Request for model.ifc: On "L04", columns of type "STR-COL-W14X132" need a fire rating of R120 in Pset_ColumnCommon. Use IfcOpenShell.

First a look at what the model holds.

```python
import ifcopenshell
import ifcopenshell.util.element

model = ifcopenshell.open("model.ifc")
print(model.schema)
storey = next(s for s in model.by_type("IfcBuildingStorey") if s.Name == "L04")
columns = [e for e in ifcopenshell.util.element.get_decomposition(storey) if e.is_a("IfcColumn")]
seen = {}
for e in columns:
    element_type = ifcopenshell.util.element.get_type(e)
    key = (element_type.Name if element_type != e and element_type else None, ifcopenshell.util.element.get_pset(e, "Pset_ColumnCommon", "FireRating"))
    seen[key] = seen.get(key, 0) + 1
for (name, value), count in sorted(seen.items(), key=str):
    print(count, "x", name, "|", value)
```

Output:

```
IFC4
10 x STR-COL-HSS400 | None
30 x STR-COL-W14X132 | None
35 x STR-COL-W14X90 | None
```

```python
import ifcopenshell
import ifcopenshell.api.pset
import ifcopenshell.util.element

model = ifcopenshell.open("model.ifc")

storey = next(s for s in model.by_type("IfcBuildingStorey") if s.Name == "L04")
columns = [e for e in ifcopenshell.util.element.get_decomposition(storey) if e.is_a("IfcColumn")]

count = 0
for e in columns:
    element_type = ifcopenshell.util.element.get_type(e)
    if element_type in (None, e) or element_type.Name != "STR-COL-W14X132":
        continue
    # add_pset returns the element's existing set when there is one.
    pset = ifcopenshell.api.pset.add_pset(model, product=e, name="Pset_ColumnCommon")
    ifcopenshell.api.pset.edit_pset(model, pset=pset, properties={"FireRating": "R120"})
    count += 1

print(count, "columns updated")

model.write("model_rev.ifc")
```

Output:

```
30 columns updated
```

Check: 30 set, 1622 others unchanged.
